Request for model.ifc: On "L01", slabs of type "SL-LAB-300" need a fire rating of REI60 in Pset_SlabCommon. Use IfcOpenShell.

First a look at what the model holds.

```python
import ifcopenshell
import ifcopenshell.util.element

model = ifcopenshell.open("model.ifc")
print(model.schema)
storey = next(s for s in model.by_type("IfcBuildingStorey") if s.Name == "L01")
slabs = [e for e in ifcopenshell.util.element.get_decomposition(storey) if e.is_a("IfcSlab")]
seen = {}
for e in slabs:
    element_type = ifcopenshell.util.element.get_type(e)
    key = (element_type.Name if element_type != e and element_type else None, ifcopenshell.util.element.get_pset(e, "Pset_SlabCommon", "FireRating"))
    seen[key] = seen.get(key, 0) + 1
for (name, value), count in sorted(seen.items(), key=str):
    print(count, "x", name, "|", value)
```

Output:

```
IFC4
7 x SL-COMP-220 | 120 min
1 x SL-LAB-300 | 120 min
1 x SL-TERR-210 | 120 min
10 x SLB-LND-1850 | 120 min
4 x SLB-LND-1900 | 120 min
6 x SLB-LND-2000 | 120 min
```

```python
import ifcopenshell
import ifcopenshell.api.pset
import ifcopenshell.util.element

model = ifcopenshell.open("model.ifc")

storey = next(s for s in model.by_type("IfcBuildingStorey") if s.Name == "L01")
slabs = [e for e in ifcopenshell.util.element.get_decomposition(storey) if e.is_a("IfcSlab")]

count = 0
for e in slabs:
    element_type = ifcopenshell.util.element.get_type(e)
    if element_type in (None, e) or element_type.Name != "SL-LAB-300":
        continue
    # add_pset returns the element's existing set when there is one.
    pset = ifcopenshell.api.pset.add_pset(model, product=e, name="Pset_SlabCommon")
    ifcopenshell.api.pset.edit_pset(model, pset=pset, properties={"FireRating": "REI60"})
    count += 1

print(count, "slabs updated")

model.write("model-out.ifc")
```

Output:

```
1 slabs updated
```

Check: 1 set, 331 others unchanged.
